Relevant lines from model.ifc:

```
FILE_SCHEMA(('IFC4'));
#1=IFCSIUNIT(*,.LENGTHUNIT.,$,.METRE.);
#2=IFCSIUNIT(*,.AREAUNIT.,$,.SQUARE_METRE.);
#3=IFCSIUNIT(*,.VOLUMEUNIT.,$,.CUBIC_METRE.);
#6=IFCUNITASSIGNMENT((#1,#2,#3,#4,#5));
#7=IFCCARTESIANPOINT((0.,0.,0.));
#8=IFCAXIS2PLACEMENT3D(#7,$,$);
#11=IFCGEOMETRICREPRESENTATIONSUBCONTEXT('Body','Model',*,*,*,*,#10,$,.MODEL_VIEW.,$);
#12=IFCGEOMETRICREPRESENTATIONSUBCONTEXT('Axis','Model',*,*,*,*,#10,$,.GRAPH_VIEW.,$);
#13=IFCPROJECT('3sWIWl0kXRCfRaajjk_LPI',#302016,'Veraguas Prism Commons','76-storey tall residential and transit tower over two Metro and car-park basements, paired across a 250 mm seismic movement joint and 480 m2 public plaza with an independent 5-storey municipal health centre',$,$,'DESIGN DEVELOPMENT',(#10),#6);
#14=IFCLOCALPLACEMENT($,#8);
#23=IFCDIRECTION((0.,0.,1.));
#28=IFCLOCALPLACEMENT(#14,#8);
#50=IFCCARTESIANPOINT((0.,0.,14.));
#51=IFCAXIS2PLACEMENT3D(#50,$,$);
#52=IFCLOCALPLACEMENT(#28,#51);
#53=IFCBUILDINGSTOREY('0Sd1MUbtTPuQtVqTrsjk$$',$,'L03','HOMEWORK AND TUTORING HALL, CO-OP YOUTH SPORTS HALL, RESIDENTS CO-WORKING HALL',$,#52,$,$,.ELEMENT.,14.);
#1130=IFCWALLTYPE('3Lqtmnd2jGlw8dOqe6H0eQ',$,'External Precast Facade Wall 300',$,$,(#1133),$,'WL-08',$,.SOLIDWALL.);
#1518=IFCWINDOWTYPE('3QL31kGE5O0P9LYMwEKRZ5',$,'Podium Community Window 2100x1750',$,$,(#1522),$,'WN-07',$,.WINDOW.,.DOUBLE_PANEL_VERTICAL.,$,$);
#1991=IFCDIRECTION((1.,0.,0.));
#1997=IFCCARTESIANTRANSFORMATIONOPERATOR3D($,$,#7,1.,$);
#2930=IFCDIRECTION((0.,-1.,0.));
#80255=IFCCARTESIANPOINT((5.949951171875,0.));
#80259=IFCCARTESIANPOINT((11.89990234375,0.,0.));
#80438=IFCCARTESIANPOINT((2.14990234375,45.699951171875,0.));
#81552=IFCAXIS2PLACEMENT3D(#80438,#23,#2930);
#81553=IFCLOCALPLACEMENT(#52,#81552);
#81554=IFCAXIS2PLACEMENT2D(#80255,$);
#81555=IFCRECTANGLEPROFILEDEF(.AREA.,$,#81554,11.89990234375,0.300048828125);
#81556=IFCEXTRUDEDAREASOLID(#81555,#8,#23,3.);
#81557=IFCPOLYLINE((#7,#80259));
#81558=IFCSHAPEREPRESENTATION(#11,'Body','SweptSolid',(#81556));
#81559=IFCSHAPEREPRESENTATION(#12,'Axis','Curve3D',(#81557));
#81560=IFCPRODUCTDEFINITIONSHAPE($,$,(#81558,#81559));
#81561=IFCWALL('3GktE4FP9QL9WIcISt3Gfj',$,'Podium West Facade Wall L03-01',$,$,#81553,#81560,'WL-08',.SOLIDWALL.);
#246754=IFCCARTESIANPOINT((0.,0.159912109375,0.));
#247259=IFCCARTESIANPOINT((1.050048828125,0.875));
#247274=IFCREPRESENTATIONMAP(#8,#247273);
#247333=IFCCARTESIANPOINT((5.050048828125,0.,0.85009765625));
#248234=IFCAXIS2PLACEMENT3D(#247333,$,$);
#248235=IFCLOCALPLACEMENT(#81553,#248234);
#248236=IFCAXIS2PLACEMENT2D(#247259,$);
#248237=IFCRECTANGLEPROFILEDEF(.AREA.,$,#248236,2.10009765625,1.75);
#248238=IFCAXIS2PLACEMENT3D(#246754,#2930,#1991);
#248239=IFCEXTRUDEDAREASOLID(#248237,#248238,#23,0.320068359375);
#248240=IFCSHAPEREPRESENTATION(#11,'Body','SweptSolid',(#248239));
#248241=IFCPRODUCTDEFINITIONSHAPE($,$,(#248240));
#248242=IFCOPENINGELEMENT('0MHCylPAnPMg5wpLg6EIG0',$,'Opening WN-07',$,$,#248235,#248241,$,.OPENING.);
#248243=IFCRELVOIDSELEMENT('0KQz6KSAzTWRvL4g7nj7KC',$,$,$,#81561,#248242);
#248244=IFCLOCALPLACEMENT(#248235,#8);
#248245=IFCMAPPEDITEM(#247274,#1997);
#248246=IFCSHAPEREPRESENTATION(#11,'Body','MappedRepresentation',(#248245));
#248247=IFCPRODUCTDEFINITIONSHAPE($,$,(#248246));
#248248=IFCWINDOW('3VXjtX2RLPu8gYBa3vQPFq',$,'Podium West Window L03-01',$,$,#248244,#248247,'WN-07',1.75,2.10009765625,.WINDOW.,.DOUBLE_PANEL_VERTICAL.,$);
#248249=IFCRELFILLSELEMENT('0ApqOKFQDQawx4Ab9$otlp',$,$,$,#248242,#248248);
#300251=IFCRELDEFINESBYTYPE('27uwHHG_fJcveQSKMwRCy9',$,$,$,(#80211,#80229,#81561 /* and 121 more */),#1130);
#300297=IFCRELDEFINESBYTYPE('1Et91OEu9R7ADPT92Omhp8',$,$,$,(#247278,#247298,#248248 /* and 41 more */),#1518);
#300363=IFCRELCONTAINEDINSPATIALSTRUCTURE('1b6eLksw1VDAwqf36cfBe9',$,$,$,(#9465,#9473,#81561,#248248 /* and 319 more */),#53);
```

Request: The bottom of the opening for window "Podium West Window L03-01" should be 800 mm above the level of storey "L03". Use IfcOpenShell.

```python
import numpy as np
import ifcopenshell
import ifcopenshell.api.geometry
import ifcopenshell.geom
import ifcopenshell.util.element
import ifcopenshell.util.placement
import ifcopenshell.util.shape
import ifcopenshell.util.unit

model = ifcopenshell.open("model.ifc")
unit_scale = ifcopenshell.util.unit.calculate_unit_scale(model)

window = model.by_guid("3VXjtX2RLPu8gYBa3vQPFq")
opening = window.FillsVoids[0].RelatingOpeningElement
storey = ifcopenshell.util.element.get_container(window, ifc_class="IfcBuildingStorey")
level = ifcopenshell.util.placement.get_local_placement(storey.ObjectPlacement)[2, 3]

# The opening's origin need not be at the sill, so measure its lowest point.
shape = ifcopenshell.geom.create_shape(ifcopenshell.geom.settings(), opening)
bottom = ifcopenshell.util.shape.get_shape_bottom_elevation(shape, shape.geometry) / unit_scale
dz = level + 0.8 / unit_scale - bottom

shift = np.array([0.0, 0.0, dz])
# The window is placed relative to its opening, so it follows when the opening moves.
matrix = ifcopenshell.util.placement.get_local_placement(opening.ObjectPlacement)
matrix[:3, 3] += shift
ifcopenshell.api.geometry.edit_object_placement(
    model, product=opening, matrix=matrix, is_si=False, should_transform_children=True
)

print(f"moved by {dz * unit_scale:+.3f} m")

model.write("model_v2.ifc")
```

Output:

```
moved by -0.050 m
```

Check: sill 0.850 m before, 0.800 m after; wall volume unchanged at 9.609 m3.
